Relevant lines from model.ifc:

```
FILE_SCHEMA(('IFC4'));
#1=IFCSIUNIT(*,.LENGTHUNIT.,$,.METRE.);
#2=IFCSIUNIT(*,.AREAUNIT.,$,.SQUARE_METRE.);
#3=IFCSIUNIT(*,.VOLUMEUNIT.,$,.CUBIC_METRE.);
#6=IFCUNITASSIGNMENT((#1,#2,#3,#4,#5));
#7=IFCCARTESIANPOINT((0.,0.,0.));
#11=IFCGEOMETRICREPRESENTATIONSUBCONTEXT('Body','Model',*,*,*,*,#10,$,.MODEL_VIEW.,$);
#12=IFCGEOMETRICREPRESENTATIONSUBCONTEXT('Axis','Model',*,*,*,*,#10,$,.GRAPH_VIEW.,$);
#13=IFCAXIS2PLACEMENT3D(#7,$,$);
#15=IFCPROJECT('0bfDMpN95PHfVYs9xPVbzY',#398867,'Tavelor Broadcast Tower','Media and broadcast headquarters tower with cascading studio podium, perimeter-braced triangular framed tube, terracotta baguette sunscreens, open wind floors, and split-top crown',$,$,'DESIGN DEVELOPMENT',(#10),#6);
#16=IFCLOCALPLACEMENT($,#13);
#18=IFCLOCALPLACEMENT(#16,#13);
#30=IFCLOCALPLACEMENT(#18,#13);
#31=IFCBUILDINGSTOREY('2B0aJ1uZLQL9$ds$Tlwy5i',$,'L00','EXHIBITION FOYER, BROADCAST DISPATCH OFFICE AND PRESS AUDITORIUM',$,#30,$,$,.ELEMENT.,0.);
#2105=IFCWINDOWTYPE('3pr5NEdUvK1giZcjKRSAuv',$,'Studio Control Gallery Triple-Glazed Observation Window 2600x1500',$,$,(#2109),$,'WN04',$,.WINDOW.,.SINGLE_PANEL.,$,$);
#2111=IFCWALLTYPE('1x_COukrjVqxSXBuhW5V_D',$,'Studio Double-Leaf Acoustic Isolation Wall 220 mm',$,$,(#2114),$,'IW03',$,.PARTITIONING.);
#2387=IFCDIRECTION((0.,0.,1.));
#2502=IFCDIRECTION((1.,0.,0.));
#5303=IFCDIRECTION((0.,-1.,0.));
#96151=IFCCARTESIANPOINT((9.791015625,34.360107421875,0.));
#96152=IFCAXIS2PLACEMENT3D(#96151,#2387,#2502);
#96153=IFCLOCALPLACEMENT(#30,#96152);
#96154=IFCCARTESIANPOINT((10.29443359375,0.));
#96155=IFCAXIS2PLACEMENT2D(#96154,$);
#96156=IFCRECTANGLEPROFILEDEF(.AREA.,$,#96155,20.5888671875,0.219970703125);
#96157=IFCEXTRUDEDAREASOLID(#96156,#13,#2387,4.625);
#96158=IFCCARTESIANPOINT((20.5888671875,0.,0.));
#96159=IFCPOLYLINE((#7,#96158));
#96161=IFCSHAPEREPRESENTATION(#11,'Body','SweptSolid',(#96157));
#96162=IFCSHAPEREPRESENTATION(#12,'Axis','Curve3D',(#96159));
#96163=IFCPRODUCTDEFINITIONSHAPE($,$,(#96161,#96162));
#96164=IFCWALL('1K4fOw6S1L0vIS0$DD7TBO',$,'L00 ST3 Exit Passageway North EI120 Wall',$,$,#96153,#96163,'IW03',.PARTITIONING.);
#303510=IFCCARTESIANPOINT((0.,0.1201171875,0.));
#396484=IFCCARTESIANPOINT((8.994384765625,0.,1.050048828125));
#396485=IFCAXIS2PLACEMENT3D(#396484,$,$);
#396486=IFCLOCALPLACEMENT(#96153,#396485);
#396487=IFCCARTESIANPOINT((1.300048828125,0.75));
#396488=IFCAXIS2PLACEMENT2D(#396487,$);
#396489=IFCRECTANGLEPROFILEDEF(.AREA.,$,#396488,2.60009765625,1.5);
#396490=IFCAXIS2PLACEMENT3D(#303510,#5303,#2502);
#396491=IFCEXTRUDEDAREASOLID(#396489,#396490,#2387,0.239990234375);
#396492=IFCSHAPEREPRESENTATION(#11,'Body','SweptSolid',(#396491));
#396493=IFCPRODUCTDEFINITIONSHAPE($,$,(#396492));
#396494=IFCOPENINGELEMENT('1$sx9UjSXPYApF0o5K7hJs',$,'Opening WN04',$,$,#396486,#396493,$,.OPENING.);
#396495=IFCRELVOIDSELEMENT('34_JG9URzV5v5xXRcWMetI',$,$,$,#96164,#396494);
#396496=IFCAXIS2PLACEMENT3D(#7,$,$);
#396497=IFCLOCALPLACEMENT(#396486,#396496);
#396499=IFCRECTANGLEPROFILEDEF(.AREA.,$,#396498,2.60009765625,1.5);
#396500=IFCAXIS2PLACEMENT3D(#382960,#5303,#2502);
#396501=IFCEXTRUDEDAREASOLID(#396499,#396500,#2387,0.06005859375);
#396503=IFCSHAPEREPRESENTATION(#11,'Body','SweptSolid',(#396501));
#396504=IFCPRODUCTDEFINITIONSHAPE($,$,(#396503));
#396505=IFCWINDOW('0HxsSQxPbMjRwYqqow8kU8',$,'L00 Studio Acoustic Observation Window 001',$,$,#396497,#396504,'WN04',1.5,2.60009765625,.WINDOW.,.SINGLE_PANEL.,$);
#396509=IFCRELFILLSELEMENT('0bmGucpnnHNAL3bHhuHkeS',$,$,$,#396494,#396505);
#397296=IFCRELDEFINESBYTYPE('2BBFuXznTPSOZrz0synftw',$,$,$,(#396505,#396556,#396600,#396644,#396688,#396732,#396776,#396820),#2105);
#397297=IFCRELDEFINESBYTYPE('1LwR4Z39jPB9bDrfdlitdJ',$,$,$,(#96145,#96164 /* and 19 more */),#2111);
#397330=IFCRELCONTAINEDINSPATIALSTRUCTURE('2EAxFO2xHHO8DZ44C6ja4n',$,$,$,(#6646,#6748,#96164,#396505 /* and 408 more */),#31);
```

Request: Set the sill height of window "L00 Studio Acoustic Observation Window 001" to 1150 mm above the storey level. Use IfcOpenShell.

```python
import numpy as np
import ifcopenshell
import ifcopenshell.api.geometry
import ifcopenshell.geom
import ifcopenshell.util.element
import ifcopenshell.util.placement
import ifcopenshell.util.shape
import ifcopenshell.util.unit

model = ifcopenshell.open("model.ifc")
unit_scale = ifcopenshell.util.unit.calculate_unit_scale(model)

window = model.by_guid("0HxsSQxPbMjRwYqqow8kU8")
opening = window.FillsVoids[0].RelatingOpeningElement
storey = ifcopenshell.util.element.get_container(window, ifc_class="IfcBuildingStorey")
level = ifcopenshell.util.placement.get_local_placement(storey.ObjectPlacement)[2, 3]

# The opening's origin need not be at the sill, so measure its lowest point.
shape = ifcopenshell.geom.create_shape(ifcopenshell.geom.settings(), opening)
bottom = ifcopenshell.util.shape.get_shape_bottom_elevation(shape, shape.geometry) / unit_scale
dz = level + 1.15 / unit_scale - bottom

shift = np.array([0.0, 0.0, dz])
# The window is placed relative to its opening, so it follows when the opening moves.
matrix = ifcopenshell.util.placement.get_local_placement(opening.ObjectPlacement)
matrix[:3, 3] += shift
ifcopenshell.api.geometry.edit_object_placement(
    model, product=opening, matrix=matrix, is_si=False, should_transform_children=True
)

print(f"moved by {dz * unit_scale:+.3f} m")

model.write("model_v2.ifc")
```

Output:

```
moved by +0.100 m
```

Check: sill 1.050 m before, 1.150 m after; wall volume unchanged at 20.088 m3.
